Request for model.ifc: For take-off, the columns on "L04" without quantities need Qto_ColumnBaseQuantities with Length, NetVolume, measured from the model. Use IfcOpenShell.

First a look at what the model holds.

```python
import ifcopenshell
import ifcopenshell.util.element
import ifcopenshell.util.unit

model = ifcopenshell.open("model.ifc")
print(model.schema)
for unit_type in ("LENGTHUNIT", "AREAUNIT", "VOLUMEUNIT"):
    print(unit_type, ifcopenshell.util.unit.calculate_unit_scale(model, unit_type))
storey = next(s for s in model.by_type("IfcBuildingStorey") if s.Name == "L04")
columns = [e for e in ifcopenshell.util.element.get_decomposition(storey) if e.is_a("IfcColumn")]
for e in sorted(columns, key=lambda e: e.id()):
    print(e.id(), e.is_a(), e.Name, list(ifcopenshell.util.element.get_psets(e, qtos_only=True)), sep=" | ")
```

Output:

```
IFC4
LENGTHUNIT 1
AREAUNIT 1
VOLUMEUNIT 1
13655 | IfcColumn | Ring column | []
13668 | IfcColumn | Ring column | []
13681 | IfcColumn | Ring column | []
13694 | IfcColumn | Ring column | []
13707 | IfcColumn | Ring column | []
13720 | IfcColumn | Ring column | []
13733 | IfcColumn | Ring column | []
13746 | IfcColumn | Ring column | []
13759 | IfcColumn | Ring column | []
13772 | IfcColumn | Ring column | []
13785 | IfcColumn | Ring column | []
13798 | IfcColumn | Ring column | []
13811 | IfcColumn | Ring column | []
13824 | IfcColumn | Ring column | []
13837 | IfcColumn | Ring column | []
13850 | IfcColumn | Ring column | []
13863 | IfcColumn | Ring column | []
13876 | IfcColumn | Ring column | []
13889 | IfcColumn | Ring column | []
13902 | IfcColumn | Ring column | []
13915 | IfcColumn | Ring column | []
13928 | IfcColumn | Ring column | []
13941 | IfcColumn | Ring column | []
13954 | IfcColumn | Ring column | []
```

```python
import ifcopenshell
import ifcopenshell.api.pset
import ifcopenshell.geom
import ifcopenshell.util.element
import ifcopenshell.util.shape
import ifcopenshell.util.unit

model = ifcopenshell.open("model.ifc")
unit_scale = ifcopenshell.util.unit.calculate_unit_scale(model)
volume_scale = ifcopenshell.util.unit.calculate_unit_scale(model, "VOLUMEUNIT")
settings = ifcopenshell.geom.settings()

storey = next(s for s in model.by_type("IfcBuildingStorey") if s.Name == "L04")
columns = [e for e in ifcopenshell.util.element.get_decomposition(storey) if e.is_a("IfcColumn")]

for e in sorted(columns, key=lambda e: e.id()):
    if ifcopenshell.util.element.get_psets(e, qtos_only=True, should_inherit=False):
        continue
    # Geometry comes back in metres, in the element's own axes.
    shape = ifcopenshell.geom.create_shape(settings, e)
    values = {
        "Length": ifcopenshell.util.shape.get_z(shape.geometry) / unit_scale,
        "NetVolume": ifcopenshell.util.shape.get_volume(shape.geometry) / volume_scale,
    }
    qto = ifcopenshell.api.pset.add_qto(model, product=e, name="Qto_ColumnBaseQuantities")
    ifcopenshell.api.pset.edit_qto(model, qto=qto, properties=values)
    print(e.id(), {k: round(v, 3) for k, v in values.items()})

model.write("model_rev.ifc")
```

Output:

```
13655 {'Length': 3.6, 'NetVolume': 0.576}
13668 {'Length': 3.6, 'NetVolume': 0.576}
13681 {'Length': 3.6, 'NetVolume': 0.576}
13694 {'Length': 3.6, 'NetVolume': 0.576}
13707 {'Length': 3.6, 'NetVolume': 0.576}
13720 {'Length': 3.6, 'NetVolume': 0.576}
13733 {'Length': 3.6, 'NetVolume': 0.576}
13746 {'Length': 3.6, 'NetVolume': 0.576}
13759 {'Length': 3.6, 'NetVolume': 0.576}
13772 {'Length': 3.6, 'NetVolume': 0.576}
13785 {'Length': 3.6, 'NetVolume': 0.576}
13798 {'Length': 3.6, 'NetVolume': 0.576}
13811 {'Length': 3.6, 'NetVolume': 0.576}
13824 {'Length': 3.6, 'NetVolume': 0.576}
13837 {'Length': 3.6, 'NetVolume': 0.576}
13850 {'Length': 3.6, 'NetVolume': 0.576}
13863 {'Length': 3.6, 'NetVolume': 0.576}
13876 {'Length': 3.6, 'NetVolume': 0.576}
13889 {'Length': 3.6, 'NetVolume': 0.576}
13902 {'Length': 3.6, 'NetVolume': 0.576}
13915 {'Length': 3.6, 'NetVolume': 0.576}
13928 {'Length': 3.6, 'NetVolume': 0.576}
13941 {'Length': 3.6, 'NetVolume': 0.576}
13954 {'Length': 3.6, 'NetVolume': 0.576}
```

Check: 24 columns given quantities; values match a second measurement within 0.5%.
